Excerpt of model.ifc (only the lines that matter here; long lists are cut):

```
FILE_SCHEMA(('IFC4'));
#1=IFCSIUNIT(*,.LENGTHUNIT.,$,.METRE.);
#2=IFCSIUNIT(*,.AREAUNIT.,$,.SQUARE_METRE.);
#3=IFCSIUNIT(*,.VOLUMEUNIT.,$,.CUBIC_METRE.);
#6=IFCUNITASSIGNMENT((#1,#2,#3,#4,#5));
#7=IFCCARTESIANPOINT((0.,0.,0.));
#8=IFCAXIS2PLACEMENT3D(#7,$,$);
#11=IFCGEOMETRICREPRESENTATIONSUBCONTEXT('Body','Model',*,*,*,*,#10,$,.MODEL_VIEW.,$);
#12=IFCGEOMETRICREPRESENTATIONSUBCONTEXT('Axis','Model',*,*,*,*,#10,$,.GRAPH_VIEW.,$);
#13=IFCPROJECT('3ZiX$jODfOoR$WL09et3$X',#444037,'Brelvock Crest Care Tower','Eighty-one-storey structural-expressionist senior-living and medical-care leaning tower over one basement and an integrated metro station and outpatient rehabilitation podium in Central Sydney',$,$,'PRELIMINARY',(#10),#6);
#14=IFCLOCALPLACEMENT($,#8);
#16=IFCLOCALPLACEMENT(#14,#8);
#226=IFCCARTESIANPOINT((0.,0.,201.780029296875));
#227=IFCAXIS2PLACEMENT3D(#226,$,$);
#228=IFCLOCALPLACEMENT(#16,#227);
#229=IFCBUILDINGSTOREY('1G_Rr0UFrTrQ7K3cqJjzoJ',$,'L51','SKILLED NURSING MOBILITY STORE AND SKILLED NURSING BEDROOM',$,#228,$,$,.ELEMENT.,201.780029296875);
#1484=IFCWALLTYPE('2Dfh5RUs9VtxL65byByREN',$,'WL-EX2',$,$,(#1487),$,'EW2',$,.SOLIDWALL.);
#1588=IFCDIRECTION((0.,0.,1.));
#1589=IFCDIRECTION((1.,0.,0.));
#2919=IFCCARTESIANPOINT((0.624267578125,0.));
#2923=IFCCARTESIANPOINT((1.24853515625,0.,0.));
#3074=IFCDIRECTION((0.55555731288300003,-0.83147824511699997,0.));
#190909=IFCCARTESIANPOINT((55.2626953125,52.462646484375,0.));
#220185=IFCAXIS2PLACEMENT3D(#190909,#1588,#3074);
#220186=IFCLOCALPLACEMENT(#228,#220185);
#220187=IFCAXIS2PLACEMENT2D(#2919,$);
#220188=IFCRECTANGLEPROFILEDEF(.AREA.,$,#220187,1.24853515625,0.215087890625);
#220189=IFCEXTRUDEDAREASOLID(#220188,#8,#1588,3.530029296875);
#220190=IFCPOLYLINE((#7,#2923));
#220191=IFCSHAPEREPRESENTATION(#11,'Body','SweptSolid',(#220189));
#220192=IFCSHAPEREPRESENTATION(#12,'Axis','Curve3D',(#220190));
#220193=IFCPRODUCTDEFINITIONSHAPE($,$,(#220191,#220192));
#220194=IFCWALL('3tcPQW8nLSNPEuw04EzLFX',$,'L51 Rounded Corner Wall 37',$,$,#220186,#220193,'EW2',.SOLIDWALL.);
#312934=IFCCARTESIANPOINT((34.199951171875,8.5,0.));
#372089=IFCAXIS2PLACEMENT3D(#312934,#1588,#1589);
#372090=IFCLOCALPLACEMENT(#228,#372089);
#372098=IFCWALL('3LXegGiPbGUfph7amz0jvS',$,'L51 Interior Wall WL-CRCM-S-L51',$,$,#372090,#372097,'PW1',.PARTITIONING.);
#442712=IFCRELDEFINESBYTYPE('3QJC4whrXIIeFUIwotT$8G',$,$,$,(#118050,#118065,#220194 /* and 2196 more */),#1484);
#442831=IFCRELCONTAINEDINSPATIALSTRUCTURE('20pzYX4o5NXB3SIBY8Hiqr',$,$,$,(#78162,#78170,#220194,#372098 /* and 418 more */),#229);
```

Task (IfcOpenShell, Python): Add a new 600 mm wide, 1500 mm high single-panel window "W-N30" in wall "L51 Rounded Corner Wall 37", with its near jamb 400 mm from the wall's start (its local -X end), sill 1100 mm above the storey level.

```python
import numpy as np
import ifcopenshell
import ifcopenshell.api.feature
import ifcopenshell.api.geometry
import ifcopenshell.api.root
import ifcopenshell.api.spatial
import ifcopenshell.geom
import ifcopenshell.util.element
import ifcopenshell.util.placement
import ifcopenshell.util.representation
import ifcopenshell.util.shape
import ifcopenshell.util.unit

model = ifcopenshell.open("model.ifc")
unit_scale = ifcopenshell.util.unit.calculate_unit_scale(model)
settings = ifcopenshell.geom.settings()


def volume(element):
    """Net volume in cubic metres, openings subtracted."""
    shape = ifcopenshell.geom.create_shape(settings, element)
    return ifcopenshell.util.shape.get_volume(shape.geometry)


wall = model.by_id(220194)
storey = ifcopenshell.util.element.get_container(wall, ifc_class="IfcBuildingStorey")
context = ifcopenshell.util.representation.get_context(model, "Model", "Body", "MODEL_VIEW")
before = volume(wall)

width, height, from_end, sill = 0.6, 1.5, 0.4, 1.1  # metres

# The wall runs along its own X axis, and the end named is its -X end.
wall_shape = ifcopenshell.geom.create_shape(settings, wall)
x, y, z = ifcopenshell.util.shape.get_vertices(wall_shape.geometry).T
start = x.min() + from_end
face, thickness = float(y.min()), float(y.max() - y.min())
wall_matrix = ifcopenshell.util.placement.get_local_placement(wall.ObjectPlacement)
level = ifcopenshell.util.placement.get_local_placement(storey.ObjectPlacement)[2, 3]


def in_wall(x, y):
    """Placement at x, y metres in the wall's axes, at sill height."""
    matrix = wall_matrix.copy()
    matrix[:, 3] = wall_matrix @ np.array([x / unit_scale, y / unit_scale, 0.0, 1.0])
    matrix[2, 3] = level + sill / unit_scale
    return matrix


# Opening: a box that overshoots both wall faces by 50 mm.
opening = ifcopenshell.api.root.create_entity(model, ifc_class="IfcOpeningElement", predefined_type="OPENING")
box = ifcopenshell.api.geometry.add_wall_representation(
    model, context=context, length=width, height=height, thickness=thickness + 0.1
)
ifcopenshell.api.geometry.assign_representation(model, product=opening, representation=box)
ifcopenshell.api.geometry.edit_object_placement(model, product=opening, matrix=in_wall(start, face - 0.05), is_si=False)
ifcopenshell.api.feature.add_feature(model, feature=opening, element=wall)

window = ifcopenshell.api.root.create_entity(model, ifc_class="IfcWindow", name="W-N30", predefined_type="WINDOW")
window.OverallWidth, window.OverallHeight = width / unit_scale, height / unit_scale
window.PartitioningType = "SINGLE_PANEL"
body = ifcopenshell.api.geometry.add_window_representation(
    model,
    context=context,
    overall_width=window.OverallWidth,
    overall_height=window.OverallHeight,
    partition_type="SINGLE_PANEL",
)
ifcopenshell.api.geometry.assign_representation(model, product=window, representation=body)
ifcopenshell.api.spatial.assign_container(model, products=[window], relating_structure=storey)
ifcopenshell.api.feature.add_filling(model, opening=opening, element=window)

# Centre the window in the wall's thickness.
ifcopenshell.api.geometry.edit_object_placement(model, product=window, matrix=in_wall(start, face), is_si=False)
window_shape = ifcopenshell.geom.create_shape(settings, window)
depth = ifcopenshell.util.shape.get_vertices(window_shape.geometry)[:, 1]
offset = face + thickness / 2 - (depth.min() + depth.max()) / 2
ifcopenshell.api.geometry.edit_object_placement(model, product=window, matrix=in_wall(start, offset), is_si=False)

after = volume(wall)

print(f"wall volume {before:.3f} -> {after:.3f} m3")

model.write("model_rev.ifc")
```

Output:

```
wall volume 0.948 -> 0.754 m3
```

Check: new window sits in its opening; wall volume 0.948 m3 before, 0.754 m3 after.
